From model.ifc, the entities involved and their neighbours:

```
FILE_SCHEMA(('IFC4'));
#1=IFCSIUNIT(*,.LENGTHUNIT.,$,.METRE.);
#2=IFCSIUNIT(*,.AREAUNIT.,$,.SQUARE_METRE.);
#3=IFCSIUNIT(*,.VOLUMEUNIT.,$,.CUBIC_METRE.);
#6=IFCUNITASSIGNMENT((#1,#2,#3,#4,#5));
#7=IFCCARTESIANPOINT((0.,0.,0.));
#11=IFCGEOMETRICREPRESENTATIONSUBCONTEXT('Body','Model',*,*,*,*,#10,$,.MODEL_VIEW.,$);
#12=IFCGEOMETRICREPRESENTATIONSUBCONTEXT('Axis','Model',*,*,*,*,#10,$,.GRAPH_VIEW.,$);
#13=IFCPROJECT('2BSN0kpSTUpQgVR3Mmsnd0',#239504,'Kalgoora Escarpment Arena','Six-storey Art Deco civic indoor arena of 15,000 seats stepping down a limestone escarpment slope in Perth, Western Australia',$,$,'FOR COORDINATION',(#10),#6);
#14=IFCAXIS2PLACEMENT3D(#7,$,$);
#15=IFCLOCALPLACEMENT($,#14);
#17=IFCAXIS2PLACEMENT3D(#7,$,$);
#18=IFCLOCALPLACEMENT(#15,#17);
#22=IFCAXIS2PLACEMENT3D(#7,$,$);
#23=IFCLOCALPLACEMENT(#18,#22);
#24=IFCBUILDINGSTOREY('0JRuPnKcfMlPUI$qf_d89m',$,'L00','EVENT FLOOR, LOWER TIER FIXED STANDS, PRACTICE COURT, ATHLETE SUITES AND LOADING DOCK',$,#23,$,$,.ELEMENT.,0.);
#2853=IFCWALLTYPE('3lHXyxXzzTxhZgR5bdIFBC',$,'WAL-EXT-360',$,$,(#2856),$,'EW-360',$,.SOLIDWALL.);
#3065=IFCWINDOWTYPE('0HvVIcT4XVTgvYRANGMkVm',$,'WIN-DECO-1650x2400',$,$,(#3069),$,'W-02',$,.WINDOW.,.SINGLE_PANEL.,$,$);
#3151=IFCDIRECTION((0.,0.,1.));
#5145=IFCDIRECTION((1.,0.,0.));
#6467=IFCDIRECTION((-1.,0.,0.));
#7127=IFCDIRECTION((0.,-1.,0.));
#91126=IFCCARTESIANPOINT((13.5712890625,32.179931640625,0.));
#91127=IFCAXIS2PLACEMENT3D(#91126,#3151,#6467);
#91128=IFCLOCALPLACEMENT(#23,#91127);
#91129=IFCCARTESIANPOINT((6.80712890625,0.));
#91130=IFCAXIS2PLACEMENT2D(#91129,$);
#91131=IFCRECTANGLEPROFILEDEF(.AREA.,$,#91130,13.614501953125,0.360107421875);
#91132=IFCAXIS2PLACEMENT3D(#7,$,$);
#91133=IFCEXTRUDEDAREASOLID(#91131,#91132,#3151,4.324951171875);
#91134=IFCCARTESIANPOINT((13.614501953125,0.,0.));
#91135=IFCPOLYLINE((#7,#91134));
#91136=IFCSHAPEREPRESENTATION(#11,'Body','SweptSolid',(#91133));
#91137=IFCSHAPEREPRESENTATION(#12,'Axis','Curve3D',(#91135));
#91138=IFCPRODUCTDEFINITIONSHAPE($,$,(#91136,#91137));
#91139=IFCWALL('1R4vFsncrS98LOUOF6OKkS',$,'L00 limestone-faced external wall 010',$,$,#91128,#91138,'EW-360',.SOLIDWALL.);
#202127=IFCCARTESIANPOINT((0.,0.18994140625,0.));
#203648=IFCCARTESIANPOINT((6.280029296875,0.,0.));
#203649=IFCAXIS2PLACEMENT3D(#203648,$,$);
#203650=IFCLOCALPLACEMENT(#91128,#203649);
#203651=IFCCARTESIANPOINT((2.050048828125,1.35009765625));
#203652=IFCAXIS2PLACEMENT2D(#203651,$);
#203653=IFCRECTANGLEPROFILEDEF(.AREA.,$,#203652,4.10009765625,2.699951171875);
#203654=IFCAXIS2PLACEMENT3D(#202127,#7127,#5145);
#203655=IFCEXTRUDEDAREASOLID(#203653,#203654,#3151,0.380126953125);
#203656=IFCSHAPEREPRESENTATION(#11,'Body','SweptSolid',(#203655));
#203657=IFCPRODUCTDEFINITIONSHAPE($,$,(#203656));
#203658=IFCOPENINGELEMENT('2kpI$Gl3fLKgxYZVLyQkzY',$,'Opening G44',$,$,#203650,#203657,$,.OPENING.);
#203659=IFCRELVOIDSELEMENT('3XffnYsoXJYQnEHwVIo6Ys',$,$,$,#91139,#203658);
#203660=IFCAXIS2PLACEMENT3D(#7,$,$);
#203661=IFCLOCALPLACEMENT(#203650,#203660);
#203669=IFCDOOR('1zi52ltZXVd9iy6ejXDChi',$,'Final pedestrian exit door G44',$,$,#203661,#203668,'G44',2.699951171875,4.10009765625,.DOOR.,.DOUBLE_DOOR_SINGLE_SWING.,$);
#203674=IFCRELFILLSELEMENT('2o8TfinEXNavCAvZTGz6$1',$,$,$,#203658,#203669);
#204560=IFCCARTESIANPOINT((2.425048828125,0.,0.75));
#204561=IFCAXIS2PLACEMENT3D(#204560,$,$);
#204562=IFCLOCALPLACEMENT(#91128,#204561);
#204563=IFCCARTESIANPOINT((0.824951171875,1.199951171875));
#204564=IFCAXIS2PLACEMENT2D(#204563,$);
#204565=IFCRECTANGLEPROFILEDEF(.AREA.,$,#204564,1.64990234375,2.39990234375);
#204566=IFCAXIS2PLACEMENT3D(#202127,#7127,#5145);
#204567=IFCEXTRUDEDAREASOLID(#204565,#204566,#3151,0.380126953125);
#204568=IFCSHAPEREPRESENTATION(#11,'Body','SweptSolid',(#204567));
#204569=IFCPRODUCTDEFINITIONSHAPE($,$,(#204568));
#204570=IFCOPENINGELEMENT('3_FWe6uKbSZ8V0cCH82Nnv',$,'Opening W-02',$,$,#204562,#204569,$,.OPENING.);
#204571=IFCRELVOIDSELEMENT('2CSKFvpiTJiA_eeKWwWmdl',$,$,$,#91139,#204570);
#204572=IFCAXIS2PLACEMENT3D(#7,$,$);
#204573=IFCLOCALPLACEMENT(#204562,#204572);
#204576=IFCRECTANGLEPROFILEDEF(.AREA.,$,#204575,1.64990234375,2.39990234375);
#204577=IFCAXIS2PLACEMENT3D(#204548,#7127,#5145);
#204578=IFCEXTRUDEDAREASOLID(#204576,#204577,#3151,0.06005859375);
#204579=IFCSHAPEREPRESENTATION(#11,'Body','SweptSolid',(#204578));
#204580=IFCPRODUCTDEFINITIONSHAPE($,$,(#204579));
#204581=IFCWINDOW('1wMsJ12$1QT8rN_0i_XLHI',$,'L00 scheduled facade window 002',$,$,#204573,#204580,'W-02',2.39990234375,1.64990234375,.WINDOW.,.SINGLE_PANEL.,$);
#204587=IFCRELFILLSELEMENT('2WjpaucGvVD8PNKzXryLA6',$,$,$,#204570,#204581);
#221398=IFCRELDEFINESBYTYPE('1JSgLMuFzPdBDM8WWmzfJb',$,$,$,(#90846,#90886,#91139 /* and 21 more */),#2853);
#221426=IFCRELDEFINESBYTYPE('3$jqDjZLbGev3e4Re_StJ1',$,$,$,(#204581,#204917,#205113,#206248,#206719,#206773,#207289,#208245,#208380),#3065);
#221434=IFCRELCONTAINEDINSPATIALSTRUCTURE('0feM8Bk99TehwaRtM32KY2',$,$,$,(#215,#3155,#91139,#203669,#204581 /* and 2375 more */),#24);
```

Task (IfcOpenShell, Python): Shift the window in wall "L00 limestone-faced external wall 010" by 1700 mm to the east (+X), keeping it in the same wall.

```python
import ifcopenshell
import ifcopenshell.api.geometry
import ifcopenshell.util.placement

model = ifcopenshell.open("model.ifc")

window = model.by_guid("1wMsJ12$1QT8rN_0i_XLHI")
opening = window.FillsVoids[0].RelatingOpeningElement
wall = opening.VoidsElements[0].RelatingBuildingElement

wall_matrix = ifcopenshell.util.placement.get_local_placement(wall.ObjectPlacement)
shift = wall_matrix[:3, 0] * -1.7
before = ifcopenshell.util.placement.get_local_placement(window.ObjectPlacement)[:3, 3].copy()

# The window is placed relative to its opening, so it follows when the opening moves.
matrix = ifcopenshell.util.placement.get_local_placement(opening.ObjectPlacement)
matrix[:3, 3] += shift
ifcopenshell.api.geometry.edit_object_placement(
    model, product=opening, matrix=matrix, is_si=False, should_transform_children=True
)

after = ifcopenshell.util.placement.get_local_placement(window.ObjectPlacement)[:3, 3]
print("window moved by", (after - before).round(3) + 0.0)

model.write("model_edited.ifc")
```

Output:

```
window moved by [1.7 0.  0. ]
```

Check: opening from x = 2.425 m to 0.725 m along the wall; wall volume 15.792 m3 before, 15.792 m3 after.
